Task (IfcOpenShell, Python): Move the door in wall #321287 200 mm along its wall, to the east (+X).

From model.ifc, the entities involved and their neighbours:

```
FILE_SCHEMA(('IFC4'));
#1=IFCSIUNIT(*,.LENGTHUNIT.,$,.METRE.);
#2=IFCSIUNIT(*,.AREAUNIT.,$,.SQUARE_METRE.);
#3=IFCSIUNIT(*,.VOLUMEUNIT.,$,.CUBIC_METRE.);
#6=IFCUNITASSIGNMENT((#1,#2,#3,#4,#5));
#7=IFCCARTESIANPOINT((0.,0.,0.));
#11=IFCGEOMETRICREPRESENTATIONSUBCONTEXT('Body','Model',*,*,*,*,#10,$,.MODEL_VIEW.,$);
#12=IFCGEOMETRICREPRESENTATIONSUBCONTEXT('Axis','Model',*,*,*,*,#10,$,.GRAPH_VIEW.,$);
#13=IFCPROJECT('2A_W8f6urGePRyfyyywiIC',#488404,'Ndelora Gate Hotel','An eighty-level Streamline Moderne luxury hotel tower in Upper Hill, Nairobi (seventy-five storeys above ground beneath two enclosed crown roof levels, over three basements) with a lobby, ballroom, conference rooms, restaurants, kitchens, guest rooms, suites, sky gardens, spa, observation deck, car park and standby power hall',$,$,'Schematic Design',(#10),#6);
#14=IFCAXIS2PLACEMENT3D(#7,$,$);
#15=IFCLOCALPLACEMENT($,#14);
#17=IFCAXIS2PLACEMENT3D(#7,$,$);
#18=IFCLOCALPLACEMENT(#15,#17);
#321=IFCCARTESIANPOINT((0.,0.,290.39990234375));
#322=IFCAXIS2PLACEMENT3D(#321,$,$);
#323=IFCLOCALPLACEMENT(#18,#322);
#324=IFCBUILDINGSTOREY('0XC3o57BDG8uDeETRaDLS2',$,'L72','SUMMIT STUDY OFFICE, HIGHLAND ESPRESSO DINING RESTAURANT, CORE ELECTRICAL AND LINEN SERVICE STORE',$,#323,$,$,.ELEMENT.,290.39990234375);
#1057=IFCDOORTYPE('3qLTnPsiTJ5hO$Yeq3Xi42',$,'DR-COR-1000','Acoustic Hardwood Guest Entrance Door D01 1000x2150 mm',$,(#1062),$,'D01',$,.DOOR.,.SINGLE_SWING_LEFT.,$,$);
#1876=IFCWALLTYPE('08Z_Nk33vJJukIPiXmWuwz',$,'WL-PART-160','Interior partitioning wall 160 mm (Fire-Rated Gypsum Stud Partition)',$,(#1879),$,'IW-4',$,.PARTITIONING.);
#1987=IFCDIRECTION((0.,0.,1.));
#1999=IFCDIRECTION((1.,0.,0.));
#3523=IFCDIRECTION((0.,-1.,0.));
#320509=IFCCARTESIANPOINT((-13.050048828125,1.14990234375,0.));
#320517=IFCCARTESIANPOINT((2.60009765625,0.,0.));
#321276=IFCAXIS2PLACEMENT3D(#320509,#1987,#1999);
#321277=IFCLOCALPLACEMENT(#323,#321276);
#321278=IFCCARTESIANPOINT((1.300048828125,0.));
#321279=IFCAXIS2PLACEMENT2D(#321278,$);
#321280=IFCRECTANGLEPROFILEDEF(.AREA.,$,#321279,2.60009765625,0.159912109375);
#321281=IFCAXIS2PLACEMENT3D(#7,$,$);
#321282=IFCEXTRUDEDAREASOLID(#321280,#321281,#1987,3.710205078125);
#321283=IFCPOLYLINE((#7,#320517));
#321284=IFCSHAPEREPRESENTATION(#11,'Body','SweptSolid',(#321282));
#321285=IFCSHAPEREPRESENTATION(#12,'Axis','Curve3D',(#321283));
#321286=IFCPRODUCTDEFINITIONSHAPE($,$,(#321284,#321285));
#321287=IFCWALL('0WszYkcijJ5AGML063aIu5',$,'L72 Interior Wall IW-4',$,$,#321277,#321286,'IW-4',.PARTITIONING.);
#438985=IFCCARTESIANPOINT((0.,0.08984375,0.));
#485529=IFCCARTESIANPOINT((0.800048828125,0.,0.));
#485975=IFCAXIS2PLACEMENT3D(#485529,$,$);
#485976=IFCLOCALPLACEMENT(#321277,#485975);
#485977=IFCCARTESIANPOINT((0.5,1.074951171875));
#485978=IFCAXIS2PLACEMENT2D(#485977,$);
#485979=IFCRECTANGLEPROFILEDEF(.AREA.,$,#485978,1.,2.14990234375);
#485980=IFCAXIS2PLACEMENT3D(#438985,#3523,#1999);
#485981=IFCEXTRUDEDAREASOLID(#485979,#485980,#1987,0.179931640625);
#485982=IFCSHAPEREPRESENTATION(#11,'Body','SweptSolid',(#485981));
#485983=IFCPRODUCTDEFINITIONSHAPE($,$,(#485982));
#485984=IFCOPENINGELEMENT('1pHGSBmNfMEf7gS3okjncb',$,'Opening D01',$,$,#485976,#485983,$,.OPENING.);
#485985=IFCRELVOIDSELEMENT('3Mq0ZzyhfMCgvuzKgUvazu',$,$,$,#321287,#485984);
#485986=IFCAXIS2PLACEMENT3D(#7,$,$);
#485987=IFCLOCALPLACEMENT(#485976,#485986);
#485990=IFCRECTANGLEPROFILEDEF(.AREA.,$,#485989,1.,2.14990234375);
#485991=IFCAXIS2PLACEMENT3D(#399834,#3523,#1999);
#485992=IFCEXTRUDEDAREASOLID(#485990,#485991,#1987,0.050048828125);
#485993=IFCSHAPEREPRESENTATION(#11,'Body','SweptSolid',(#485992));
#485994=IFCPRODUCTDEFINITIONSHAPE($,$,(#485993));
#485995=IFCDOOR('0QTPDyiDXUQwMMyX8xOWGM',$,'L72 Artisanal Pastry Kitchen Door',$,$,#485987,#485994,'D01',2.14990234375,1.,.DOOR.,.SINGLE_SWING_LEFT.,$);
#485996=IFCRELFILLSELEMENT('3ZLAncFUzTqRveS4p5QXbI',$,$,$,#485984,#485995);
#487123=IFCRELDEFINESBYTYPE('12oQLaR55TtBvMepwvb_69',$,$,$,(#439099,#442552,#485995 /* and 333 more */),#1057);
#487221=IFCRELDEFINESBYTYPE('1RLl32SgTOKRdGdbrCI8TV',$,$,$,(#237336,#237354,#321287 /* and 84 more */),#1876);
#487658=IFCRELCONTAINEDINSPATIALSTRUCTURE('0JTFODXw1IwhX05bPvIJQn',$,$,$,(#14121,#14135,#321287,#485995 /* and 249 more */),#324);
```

```python
import ifcopenshell
import ifcopenshell.api.geometry
import ifcopenshell.util.placement

model = ifcopenshell.open("model.ifc")

door = model.by_id(485995)
opening = door.FillsVoids[0].RelatingOpeningElement
wall = opening.VoidsElements[0].RelatingBuildingElement

wall_matrix = ifcopenshell.util.placement.get_local_placement(wall.ObjectPlacement)
shift = wall_matrix[:3, 0] * 0.2
before = ifcopenshell.util.placement.get_local_placement(door.ObjectPlacement)[:3, 3].copy()

# The door is placed relative to its opening, so it follows when the opening moves.
matrix = ifcopenshell.util.placement.get_local_placement(opening.ObjectPlacement)
matrix[:3, 3] += shift
ifcopenshell.api.geometry.edit_object_placement(
    model, product=opening, matrix=matrix, is_si=False, should_transform_children=True
)

after = ifcopenshell.util.placement.get_local_placement(door.ObjectPlacement)[:3, 3]
print("door moved by", (after - before).round(3) + 0.0)

model.write("model_updated.ifc")
```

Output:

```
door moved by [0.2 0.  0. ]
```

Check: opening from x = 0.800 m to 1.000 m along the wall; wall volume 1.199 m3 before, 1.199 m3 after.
